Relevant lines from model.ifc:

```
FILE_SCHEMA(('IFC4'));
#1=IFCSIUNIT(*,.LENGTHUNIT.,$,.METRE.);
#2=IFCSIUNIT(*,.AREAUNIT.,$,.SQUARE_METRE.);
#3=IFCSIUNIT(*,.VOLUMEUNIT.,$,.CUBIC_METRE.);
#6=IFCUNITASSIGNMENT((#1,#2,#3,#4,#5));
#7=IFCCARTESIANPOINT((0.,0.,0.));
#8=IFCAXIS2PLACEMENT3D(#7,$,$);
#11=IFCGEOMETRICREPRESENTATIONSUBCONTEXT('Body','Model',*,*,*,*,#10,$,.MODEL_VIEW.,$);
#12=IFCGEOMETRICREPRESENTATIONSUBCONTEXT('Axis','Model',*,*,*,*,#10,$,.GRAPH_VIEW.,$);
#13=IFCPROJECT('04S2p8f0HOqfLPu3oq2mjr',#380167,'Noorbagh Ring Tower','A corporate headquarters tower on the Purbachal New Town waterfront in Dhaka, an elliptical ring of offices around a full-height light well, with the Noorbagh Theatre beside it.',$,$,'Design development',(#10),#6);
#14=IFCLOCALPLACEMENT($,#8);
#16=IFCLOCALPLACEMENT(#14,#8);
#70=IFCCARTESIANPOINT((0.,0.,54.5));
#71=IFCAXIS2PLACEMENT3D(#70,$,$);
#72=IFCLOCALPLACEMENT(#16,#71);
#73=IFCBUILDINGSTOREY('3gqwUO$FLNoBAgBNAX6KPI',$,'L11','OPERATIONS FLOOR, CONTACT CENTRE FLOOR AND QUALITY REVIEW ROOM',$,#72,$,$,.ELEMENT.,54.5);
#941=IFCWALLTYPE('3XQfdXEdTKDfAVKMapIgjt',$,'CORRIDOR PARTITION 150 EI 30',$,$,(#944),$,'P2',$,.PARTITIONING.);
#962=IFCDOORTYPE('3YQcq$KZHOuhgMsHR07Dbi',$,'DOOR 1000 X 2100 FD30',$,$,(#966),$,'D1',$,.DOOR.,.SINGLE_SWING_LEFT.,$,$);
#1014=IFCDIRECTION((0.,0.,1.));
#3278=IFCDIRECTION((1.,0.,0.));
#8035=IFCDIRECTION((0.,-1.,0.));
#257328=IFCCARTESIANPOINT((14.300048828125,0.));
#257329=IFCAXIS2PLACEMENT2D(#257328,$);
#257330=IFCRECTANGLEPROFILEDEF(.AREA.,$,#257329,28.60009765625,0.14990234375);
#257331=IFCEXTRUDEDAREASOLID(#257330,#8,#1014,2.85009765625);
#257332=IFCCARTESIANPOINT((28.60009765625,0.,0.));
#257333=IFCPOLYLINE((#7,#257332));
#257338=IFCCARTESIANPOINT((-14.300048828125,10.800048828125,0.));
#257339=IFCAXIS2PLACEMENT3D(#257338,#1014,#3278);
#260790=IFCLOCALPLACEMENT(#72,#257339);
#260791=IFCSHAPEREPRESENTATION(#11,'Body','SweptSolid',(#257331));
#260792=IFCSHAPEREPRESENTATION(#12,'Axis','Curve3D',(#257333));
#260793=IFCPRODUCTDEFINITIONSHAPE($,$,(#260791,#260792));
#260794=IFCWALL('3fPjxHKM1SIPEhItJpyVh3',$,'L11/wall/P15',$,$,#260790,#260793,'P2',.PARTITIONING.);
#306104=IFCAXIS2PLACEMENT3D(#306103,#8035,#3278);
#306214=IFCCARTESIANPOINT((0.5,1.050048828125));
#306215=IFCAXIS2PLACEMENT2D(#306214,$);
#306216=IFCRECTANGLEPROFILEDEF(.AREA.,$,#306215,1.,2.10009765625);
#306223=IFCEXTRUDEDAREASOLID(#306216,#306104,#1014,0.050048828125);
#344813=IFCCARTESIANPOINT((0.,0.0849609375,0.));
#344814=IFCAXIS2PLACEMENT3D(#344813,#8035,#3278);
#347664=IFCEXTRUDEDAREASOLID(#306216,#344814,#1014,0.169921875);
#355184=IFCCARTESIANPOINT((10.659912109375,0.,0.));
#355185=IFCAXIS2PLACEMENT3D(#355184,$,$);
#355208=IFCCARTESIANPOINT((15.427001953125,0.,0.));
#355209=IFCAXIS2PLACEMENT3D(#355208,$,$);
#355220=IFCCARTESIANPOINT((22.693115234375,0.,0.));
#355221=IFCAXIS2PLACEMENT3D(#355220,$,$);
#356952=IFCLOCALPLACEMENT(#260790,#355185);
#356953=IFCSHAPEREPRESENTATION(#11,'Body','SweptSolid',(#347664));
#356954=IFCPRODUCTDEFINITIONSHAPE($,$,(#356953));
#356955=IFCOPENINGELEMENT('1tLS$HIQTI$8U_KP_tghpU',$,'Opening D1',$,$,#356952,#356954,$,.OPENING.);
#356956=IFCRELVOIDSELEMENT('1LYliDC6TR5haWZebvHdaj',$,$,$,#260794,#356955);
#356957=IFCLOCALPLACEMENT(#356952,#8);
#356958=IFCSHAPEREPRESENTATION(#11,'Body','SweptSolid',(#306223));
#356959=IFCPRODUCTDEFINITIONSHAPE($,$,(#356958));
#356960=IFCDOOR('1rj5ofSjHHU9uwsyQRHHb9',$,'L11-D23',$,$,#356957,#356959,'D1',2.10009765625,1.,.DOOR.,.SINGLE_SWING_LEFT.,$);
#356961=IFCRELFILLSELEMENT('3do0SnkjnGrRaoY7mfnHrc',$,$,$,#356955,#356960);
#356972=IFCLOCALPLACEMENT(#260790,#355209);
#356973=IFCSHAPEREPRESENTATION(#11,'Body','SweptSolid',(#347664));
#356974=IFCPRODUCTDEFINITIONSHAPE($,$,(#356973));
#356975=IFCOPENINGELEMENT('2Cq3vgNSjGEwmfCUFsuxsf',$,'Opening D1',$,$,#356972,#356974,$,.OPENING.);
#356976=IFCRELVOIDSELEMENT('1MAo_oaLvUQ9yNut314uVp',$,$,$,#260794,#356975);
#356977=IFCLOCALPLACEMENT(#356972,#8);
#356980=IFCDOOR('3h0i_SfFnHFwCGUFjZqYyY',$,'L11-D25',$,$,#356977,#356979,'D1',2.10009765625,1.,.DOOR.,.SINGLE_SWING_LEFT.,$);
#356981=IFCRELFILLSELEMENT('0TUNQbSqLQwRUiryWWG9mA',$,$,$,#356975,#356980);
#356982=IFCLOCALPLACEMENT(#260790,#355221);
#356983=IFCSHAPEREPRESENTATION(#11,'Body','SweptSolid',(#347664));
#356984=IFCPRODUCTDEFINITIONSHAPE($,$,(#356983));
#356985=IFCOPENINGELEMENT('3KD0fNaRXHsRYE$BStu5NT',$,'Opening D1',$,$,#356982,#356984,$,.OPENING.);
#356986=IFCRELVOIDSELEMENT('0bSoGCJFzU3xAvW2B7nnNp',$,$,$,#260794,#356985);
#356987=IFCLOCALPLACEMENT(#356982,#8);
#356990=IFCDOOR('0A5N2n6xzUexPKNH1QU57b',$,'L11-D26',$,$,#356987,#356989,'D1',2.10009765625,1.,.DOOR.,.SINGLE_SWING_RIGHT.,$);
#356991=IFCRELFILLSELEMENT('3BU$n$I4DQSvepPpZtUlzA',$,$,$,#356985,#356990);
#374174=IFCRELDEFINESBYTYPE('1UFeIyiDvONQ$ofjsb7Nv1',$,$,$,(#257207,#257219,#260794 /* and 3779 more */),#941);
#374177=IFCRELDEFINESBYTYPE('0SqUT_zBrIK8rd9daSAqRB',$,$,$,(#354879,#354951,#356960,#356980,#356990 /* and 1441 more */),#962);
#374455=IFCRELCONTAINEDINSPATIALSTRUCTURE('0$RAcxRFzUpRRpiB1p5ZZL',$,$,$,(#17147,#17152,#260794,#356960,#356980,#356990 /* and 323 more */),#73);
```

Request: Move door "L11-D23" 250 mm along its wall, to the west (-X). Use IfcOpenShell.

```python
import ifcopenshell
import ifcopenshell.api.geometry
import ifcopenshell.util.placement

model = ifcopenshell.open("model.ifc")

door = model.by_guid("1rj5ofSjHHU9uwsyQRHHb9")
opening = door.FillsVoids[0].RelatingOpeningElement
wall = opening.VoidsElements[0].RelatingBuildingElement

wall_matrix = ifcopenshell.util.placement.get_local_placement(wall.ObjectPlacement)
shift = wall_matrix[:3, 0] * -0.25
before = ifcopenshell.util.placement.get_local_placement(door.ObjectPlacement)[:3, 3].copy()

# The door is placed relative to its opening, so it follows when the opening moves.
matrix = ifcopenshell.util.placement.get_local_placement(opening.ObjectPlacement)
matrix[:3, 3] += shift
ifcopenshell.api.geometry.edit_object_placement(
    model, product=opening, matrix=matrix, is_si=False, should_transform_children=True
)

after = ifcopenshell.util.placement.get_local_placement(door.ObjectPlacement)[:3, 3]
print("door moved by", (after - before).round(3) + 0.0)

model.write("model-out.ifc")
```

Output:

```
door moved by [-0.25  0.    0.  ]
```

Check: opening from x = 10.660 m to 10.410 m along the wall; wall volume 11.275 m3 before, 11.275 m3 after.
